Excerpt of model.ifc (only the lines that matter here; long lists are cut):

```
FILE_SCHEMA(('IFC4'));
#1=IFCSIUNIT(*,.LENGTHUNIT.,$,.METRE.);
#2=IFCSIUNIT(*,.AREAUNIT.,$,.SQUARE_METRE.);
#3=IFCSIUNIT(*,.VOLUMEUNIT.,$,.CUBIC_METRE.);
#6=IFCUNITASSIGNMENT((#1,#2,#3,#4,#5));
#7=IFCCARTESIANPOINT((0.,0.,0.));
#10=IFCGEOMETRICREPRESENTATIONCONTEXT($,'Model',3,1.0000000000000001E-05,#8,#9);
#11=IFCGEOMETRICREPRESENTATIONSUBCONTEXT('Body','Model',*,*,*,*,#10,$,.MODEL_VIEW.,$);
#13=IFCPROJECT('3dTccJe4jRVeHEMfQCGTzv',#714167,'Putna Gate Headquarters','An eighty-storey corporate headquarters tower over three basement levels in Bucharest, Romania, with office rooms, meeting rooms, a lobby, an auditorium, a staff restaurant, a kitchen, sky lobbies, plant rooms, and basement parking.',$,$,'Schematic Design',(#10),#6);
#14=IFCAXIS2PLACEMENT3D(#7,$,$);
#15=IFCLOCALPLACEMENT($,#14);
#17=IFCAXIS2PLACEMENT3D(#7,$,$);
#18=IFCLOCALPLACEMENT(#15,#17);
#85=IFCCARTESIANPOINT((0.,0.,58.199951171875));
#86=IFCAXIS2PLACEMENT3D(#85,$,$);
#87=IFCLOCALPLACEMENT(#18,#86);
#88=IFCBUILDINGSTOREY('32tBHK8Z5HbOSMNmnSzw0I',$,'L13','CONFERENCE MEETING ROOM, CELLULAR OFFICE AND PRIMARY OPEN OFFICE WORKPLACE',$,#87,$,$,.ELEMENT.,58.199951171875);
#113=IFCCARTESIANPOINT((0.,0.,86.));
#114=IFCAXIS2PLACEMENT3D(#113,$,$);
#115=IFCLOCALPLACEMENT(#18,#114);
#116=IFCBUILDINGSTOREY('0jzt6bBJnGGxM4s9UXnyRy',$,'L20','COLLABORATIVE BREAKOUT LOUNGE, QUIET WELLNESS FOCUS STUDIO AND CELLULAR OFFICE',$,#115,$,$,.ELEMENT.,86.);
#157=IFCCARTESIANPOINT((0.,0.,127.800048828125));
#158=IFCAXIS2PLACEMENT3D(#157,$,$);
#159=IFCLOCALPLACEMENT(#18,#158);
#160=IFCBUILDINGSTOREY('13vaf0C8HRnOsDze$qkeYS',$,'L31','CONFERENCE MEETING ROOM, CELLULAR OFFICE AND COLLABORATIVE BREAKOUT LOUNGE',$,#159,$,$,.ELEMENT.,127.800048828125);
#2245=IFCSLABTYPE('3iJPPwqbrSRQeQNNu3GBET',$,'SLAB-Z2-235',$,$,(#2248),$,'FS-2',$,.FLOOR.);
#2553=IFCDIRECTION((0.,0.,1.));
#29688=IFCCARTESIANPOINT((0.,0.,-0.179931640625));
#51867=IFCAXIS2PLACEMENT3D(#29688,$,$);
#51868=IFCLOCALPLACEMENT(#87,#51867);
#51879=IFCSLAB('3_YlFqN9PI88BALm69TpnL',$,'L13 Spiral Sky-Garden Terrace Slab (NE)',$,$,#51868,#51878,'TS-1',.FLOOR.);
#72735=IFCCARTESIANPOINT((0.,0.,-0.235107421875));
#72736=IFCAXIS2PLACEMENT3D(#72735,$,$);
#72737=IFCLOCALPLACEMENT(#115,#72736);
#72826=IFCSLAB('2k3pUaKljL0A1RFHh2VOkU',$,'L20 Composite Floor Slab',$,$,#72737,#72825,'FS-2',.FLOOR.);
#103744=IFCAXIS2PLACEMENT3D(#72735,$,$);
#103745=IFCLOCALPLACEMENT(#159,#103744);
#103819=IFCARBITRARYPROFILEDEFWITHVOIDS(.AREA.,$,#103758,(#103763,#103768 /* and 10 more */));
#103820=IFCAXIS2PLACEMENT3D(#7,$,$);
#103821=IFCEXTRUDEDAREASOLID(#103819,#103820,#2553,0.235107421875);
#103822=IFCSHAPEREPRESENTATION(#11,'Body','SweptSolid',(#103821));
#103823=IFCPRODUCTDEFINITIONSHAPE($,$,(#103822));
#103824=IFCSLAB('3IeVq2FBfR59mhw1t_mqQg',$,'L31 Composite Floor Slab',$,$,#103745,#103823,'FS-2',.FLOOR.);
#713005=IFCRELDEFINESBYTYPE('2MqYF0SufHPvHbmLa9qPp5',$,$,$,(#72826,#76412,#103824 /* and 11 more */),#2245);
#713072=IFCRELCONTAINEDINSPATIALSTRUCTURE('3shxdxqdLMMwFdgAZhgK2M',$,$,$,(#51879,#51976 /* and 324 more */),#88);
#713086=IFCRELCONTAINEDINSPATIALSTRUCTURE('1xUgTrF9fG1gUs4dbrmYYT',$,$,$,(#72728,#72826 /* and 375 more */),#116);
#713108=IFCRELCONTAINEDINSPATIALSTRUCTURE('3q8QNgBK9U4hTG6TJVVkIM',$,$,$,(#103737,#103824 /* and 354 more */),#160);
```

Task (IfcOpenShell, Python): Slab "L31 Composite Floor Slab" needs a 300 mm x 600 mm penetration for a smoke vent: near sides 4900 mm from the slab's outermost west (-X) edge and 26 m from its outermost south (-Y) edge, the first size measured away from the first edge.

```python
import numpy as np
import ifcopenshell
import ifcopenshell.api.feature
import ifcopenshell.api.geometry
import ifcopenshell.api.root
import ifcopenshell.geom
import ifcopenshell.util.placement
import ifcopenshell.util.representation
import ifcopenshell.util.shape
import ifcopenshell.util.unit

model = ifcopenshell.open("model.ifc")
unit_scale = ifcopenshell.util.unit.calculate_unit_scale(model)
settings = ifcopenshell.geom.settings()


def volume(element):
    """Net volume in cubic metres, openings subtracted."""
    shape = ifcopenshell.geom.create_shape(settings, element)
    return ifcopenshell.util.shape.get_volume(shape.geometry)


slab = model.by_guid("3IeVq2FBfR59mhw1t_mqQg")
before = volume(slab)

# Extent in the slab's own axes, in metres. The edges named are its -X and -Y sides.
slab_shape = ifcopenshell.geom.create_shape(settings, slab)
vertices = ifcopenshell.util.shape.get_vertices(slab_shape.geometry)
x_min, y_min, bottom = vertices.min(axis=0)
top = vertices[:, 2].max()

opening = ifcopenshell.api.root.create_entity(model, ifc_class="IfcOpeningElement", name="Smoke vent opening", predefined_type="OPENING")
context = ifcopenshell.util.representation.get_context(model, "Model", "Body", "MODEL_VIEW")
width, depth = 0.3, 0.6
outline = [(0.0, 0.0), (width, 0.0), (width, depth), (0.0, depth), (0.0, 0.0)]
# Overshoot both faces by 50 mm so the cut is clean.
shape = ifcopenshell.api.geometry.add_slab_representation(
    model, context=context, depth=top - bottom + 0.1, polyline=outline
)
ifcopenshell.api.geometry.assign_representation(model, product=opening, representation=shape)

matrix = ifcopenshell.util.placement.get_local_placement(slab.ObjectPlacement)
matrix[:, 3] = matrix @ np.append(np.array([x_min + 4.9, y_min + 26, bottom - 0.05]) / unit_scale, 1.0)
ifcopenshell.api.geometry.edit_object_placement(model, product=opening, matrix=matrix, is_si=False)
ifcopenshell.api.feature.add_feature(model, feature=opening, element=slab)

after = volume(slab)

print(f"slab volume {before:.3f} -> {after:.3f} m3")

model.write("model_v2.ifc")
```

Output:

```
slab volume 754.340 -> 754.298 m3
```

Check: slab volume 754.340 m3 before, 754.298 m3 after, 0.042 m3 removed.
